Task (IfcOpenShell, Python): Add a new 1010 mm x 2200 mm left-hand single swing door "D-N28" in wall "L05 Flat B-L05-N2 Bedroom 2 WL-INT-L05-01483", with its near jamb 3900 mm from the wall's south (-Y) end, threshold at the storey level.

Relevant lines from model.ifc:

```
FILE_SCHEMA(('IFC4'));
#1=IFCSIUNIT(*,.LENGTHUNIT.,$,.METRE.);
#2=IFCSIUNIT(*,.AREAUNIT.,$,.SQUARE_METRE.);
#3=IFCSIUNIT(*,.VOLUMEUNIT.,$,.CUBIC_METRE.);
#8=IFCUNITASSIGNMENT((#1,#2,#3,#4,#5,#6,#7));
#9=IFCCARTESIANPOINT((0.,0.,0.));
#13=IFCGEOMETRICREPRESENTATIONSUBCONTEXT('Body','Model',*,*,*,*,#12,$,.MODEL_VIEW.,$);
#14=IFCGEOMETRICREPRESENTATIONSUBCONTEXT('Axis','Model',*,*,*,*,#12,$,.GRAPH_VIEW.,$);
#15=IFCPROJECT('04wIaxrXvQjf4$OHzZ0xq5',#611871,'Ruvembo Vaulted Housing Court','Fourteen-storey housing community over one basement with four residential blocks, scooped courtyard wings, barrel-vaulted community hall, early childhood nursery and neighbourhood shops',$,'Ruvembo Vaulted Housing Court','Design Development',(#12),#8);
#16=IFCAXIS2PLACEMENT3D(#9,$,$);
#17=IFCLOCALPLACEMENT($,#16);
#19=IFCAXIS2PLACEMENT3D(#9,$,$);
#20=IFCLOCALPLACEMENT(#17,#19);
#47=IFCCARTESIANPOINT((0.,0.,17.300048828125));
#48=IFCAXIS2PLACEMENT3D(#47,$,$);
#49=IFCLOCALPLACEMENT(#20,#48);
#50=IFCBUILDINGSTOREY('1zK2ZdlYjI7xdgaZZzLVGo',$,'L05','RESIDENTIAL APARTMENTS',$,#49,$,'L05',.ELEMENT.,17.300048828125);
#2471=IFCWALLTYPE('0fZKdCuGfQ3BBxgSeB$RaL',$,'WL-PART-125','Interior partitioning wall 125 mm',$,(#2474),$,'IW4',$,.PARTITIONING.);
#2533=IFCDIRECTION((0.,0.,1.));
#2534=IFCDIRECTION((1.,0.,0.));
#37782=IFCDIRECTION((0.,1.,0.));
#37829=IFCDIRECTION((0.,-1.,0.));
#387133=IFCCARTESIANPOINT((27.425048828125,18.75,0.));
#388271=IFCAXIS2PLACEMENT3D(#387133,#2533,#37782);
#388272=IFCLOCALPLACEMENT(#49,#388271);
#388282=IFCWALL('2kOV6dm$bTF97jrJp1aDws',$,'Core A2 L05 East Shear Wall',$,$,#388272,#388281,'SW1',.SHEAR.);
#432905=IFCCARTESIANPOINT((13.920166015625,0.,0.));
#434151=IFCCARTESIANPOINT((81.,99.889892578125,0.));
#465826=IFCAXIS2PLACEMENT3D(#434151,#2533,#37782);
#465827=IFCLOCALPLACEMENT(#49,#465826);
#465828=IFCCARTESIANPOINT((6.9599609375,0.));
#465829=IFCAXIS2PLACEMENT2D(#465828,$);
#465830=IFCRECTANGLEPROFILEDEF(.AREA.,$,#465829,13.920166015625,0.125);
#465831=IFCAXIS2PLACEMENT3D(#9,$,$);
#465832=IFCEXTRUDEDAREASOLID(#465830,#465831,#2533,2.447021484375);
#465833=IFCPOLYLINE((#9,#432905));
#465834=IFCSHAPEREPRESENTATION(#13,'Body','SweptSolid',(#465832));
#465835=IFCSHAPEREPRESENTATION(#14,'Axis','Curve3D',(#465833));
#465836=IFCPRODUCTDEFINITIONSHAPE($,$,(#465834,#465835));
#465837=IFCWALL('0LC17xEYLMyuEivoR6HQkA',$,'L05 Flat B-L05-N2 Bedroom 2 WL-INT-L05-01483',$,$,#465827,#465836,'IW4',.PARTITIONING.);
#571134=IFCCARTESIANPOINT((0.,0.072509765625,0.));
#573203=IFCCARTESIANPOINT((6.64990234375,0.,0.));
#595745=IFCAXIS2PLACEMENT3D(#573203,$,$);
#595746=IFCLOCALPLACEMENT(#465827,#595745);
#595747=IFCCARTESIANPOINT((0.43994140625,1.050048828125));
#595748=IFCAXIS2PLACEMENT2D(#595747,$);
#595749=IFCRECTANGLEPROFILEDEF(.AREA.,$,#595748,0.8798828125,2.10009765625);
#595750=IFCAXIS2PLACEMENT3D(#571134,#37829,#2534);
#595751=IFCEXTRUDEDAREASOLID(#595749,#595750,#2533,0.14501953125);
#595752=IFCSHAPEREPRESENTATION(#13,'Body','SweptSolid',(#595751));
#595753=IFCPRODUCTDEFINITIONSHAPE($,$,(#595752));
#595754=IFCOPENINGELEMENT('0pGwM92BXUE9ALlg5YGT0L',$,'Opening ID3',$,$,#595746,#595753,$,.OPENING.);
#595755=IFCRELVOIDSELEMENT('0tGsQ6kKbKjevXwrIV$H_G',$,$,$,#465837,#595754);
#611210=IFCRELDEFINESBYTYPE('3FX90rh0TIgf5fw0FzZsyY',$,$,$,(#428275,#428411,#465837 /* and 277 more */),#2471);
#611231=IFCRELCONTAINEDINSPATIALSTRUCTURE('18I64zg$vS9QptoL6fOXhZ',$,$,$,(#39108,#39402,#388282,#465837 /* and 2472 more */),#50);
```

```python
import numpy as np
import ifcopenshell
import ifcopenshell.api.feature
import ifcopenshell.api.geometry
import ifcopenshell.api.root
import ifcopenshell.api.spatial
import ifcopenshell.geom
import ifcopenshell.util.element
import ifcopenshell.util.placement
import ifcopenshell.util.representation
import ifcopenshell.util.shape
import ifcopenshell.util.unit

model = ifcopenshell.open("model.ifc")
unit_scale = ifcopenshell.util.unit.calculate_unit_scale(model)
settings = ifcopenshell.geom.settings()


def volume(element):
    """Net volume in cubic metres, openings subtracted."""
    shape = ifcopenshell.geom.create_shape(settings, element)
    return ifcopenshell.util.shape.get_volume(shape.geometry)


wall = model.by_guid("0LC17xEYLMyuEivoR6HQkA")
storey = ifcopenshell.util.element.get_container(wall, ifc_class="IfcBuildingStorey")
context = ifcopenshell.util.representation.get_context(model, "Model", "Body", "MODEL_VIEW")
before = volume(wall)

width, height, from_end, sill = 1.01, 2.2, 3.9, 0.0  # metres

# The wall runs along its own X axis, and the end named is its -X end.
wall_shape = ifcopenshell.geom.create_shape(settings, wall)
x, y, z = ifcopenshell.util.shape.get_vertices(wall_shape.geometry).T
start = x.min() + from_end
face, thickness = float(y.min()), float(y.max() - y.min())
wall_matrix = ifcopenshell.util.placement.get_local_placement(wall.ObjectPlacement)
level = ifcopenshell.util.placement.get_local_placement(storey.ObjectPlacement)[2, 3]


def in_wall(x, y):
    """Placement at x, y metres in the wall's axes, at sill height."""
    matrix = wall_matrix.copy()
    matrix[:, 3] = wall_matrix @ np.array([x / unit_scale, y / unit_scale, 0.0, 1.0])
    matrix[2, 3] = level + sill / unit_scale
    return matrix


# Opening: a box that overshoots both wall faces by 50 mm.
opening = ifcopenshell.api.root.create_entity(model, ifc_class="IfcOpeningElement", predefined_type="OPENING")
box = ifcopenshell.api.geometry.add_wall_representation(
    model, context=context, length=width, height=height, thickness=thickness + 0.1
)
ifcopenshell.api.geometry.assign_representation(model, product=opening, representation=box)
ifcopenshell.api.geometry.edit_object_placement(model, product=opening, matrix=in_wall(start, face - 0.05), is_si=False)
ifcopenshell.api.feature.add_feature(model, feature=opening, element=wall)

door = ifcopenshell.api.root.create_entity(model, ifc_class="IfcDoor", name="D-N28", predefined_type="DOOR")
door.OverallWidth, door.OverallHeight = width / unit_scale, height / unit_scale
door.OperationType = "SINGLE_SWING_LEFT"
body = ifcopenshell.api.geometry.add_door_representation(
    model,
    context=context,
    overall_width=door.OverallWidth,
    overall_height=door.OverallHeight,
    operation_type="SINGLE_SWING_LEFT",
    lining_properties={"LiningDepth": thickness / unit_scale, "ThresholdDepth": thickness / unit_scale},
)
ifcopenshell.api.geometry.assign_representation(model, product=door, representation=body)
ifcopenshell.api.spatial.assign_container(model, products=[door], relating_structure=storey)
ifcopenshell.api.feature.add_filling(model, opening=opening, element=door)

# The lining spans the wall, so the door starts at the wall face.
ifcopenshell.api.geometry.edit_object_placement(model, product=door, matrix=in_wall(start, face), is_si=False)

after = volume(wall)

print(f"wall volume {before:.3f} -> {after:.3f} m3")

model.write("model_updated.ifc")
```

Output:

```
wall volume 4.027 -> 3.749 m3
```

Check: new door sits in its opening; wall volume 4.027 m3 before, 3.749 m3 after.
